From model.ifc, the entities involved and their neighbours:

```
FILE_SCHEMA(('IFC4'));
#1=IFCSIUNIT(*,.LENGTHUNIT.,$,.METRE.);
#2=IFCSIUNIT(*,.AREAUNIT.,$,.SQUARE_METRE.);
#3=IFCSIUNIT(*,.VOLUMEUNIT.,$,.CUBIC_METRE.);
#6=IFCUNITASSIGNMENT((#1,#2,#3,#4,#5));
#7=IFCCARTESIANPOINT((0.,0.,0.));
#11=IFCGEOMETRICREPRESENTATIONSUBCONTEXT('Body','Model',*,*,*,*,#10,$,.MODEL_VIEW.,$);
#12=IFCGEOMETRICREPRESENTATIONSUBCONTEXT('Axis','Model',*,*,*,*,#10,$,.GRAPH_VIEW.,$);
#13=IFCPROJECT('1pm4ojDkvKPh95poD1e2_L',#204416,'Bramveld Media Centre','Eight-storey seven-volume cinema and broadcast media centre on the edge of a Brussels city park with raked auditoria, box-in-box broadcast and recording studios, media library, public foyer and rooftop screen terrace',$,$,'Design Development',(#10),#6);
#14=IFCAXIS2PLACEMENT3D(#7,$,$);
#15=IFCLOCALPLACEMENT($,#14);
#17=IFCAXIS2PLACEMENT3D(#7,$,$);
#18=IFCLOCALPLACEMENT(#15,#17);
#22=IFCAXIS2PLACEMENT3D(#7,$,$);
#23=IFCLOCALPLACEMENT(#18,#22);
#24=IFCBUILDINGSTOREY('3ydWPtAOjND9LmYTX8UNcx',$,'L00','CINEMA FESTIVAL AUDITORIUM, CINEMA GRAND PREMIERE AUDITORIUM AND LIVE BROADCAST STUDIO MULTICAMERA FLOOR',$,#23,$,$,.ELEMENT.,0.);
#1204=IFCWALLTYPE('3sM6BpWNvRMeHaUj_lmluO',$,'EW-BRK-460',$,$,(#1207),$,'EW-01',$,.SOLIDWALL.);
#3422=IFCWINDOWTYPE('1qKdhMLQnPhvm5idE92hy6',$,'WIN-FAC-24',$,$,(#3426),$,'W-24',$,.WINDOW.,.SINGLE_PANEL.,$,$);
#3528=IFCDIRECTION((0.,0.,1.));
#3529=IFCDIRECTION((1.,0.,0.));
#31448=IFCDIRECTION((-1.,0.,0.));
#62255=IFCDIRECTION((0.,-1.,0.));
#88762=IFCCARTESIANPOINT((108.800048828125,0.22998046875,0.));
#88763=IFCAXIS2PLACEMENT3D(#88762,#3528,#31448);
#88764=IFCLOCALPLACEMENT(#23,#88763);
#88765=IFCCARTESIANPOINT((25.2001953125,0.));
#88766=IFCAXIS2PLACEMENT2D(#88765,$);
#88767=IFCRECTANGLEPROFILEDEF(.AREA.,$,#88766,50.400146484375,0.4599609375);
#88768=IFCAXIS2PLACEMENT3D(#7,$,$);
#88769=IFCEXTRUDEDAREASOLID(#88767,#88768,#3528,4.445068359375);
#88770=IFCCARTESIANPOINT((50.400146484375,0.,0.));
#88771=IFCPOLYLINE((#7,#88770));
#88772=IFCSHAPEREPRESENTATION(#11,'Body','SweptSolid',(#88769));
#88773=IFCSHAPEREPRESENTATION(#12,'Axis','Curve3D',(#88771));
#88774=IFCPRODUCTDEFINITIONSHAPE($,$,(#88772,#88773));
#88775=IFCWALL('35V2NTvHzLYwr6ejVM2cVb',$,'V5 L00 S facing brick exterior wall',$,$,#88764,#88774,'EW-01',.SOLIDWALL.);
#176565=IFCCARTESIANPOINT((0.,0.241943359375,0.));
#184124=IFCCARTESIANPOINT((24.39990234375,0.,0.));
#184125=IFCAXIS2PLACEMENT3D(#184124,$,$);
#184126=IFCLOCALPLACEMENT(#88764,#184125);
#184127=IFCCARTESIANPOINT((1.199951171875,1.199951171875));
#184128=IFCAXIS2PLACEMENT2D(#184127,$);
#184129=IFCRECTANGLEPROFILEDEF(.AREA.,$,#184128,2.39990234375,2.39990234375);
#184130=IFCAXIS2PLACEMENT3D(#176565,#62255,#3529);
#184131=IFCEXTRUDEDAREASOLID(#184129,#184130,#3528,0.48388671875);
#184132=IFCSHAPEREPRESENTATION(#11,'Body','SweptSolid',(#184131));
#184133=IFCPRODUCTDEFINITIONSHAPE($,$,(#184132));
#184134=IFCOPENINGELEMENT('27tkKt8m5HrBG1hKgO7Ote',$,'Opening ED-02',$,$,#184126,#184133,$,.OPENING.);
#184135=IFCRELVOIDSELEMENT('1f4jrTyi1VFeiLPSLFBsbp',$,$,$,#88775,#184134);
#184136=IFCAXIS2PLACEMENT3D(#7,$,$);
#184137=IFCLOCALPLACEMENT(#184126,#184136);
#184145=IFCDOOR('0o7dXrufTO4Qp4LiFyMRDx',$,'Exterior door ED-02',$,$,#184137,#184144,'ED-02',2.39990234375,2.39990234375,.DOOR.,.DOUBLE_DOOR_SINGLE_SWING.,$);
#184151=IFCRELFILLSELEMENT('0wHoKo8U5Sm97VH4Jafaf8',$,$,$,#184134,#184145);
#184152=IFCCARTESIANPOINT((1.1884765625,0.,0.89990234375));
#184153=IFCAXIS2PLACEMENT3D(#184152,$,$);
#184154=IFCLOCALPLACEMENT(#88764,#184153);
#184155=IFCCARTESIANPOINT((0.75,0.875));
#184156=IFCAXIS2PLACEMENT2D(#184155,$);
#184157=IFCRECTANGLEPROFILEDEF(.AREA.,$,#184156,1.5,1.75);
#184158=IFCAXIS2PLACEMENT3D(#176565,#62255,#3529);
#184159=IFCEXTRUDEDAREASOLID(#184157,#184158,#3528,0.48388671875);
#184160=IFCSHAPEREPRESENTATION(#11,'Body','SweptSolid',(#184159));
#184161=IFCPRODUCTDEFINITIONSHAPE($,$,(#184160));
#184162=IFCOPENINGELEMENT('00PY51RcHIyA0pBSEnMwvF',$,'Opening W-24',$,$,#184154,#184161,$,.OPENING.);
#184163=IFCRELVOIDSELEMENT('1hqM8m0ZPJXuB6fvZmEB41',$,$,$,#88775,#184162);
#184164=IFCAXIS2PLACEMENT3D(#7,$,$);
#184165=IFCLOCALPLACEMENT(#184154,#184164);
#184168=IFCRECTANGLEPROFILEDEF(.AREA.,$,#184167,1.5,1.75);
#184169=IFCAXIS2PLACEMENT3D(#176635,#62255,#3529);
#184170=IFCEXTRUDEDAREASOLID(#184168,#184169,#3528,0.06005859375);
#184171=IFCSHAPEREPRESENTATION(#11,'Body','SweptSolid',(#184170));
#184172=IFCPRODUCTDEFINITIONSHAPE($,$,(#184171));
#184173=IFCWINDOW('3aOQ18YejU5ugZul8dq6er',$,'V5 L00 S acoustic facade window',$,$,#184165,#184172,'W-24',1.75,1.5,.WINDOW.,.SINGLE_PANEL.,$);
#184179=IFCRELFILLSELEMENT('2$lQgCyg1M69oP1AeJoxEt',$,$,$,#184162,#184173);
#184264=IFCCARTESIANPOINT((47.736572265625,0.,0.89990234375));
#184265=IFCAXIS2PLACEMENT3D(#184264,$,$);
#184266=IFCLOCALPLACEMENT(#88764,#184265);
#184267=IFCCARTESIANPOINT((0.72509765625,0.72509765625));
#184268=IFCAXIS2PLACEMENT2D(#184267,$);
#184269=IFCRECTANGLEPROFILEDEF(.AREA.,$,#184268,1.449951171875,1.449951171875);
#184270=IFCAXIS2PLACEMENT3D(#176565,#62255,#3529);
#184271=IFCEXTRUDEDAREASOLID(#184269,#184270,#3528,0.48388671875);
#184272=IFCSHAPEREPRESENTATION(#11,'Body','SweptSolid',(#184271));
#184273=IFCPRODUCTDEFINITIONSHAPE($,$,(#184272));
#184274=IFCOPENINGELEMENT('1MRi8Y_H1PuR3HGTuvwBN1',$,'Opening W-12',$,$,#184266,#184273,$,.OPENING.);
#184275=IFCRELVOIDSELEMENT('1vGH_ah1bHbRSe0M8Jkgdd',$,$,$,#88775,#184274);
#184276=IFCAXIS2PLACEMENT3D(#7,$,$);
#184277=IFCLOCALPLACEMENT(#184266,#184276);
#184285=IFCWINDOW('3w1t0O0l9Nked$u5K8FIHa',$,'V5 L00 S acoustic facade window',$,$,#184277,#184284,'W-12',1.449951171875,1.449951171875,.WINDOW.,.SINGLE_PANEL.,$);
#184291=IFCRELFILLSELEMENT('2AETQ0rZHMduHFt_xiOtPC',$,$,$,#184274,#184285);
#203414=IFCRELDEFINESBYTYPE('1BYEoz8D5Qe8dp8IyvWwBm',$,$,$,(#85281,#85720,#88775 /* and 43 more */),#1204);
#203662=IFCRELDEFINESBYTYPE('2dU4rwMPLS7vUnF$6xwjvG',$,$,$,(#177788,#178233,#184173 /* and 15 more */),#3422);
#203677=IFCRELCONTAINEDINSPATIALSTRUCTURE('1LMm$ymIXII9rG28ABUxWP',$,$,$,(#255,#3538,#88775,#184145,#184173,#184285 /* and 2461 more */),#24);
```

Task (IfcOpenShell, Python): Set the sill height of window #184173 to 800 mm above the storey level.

```python
import numpy as np
import ifcopenshell
import ifcopenshell.api.geometry
import ifcopenshell.geom
import ifcopenshell.util.element
import ifcopenshell.util.placement
import ifcopenshell.util.shape
import ifcopenshell.util.unit

model = ifcopenshell.open("model.ifc")
unit_scale = ifcopenshell.util.unit.calculate_unit_scale(model)

window = model.by_guid("3aOQ18YejU5ugZul8dq6er")
opening = window.FillsVoids[0].RelatingOpeningElement
storey = ifcopenshell.util.element.get_container(window, ifc_class="IfcBuildingStorey")
level = ifcopenshell.util.placement.get_local_placement(storey.ObjectPlacement)[2, 3]

# The opening's origin need not be at the sill, so measure its lowest point.
shape = ifcopenshell.geom.create_shape(ifcopenshell.geom.settings(), opening)
bottom = ifcopenshell.util.shape.get_shape_bottom_elevation(shape, shape.geometry) / unit_scale
dz = level + 0.8 / unit_scale - bottom

shift = np.array([0.0, 0.0, dz])
# The window is placed relative to its opening, so it follows when the opening moves.
matrix = ifcopenshell.util.placement.get_local_placement(opening.ObjectPlacement)
matrix[:3, 3] += shift
ifcopenshell.api.geometry.edit_object_placement(
    model, product=opening, matrix=matrix, is_si=False, should_transform_children=True
)

print(f"moved by {dz * unit_scale:+.3f} m")

model.write("model_v2.ifc")
```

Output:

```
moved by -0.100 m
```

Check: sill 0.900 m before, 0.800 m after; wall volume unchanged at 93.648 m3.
